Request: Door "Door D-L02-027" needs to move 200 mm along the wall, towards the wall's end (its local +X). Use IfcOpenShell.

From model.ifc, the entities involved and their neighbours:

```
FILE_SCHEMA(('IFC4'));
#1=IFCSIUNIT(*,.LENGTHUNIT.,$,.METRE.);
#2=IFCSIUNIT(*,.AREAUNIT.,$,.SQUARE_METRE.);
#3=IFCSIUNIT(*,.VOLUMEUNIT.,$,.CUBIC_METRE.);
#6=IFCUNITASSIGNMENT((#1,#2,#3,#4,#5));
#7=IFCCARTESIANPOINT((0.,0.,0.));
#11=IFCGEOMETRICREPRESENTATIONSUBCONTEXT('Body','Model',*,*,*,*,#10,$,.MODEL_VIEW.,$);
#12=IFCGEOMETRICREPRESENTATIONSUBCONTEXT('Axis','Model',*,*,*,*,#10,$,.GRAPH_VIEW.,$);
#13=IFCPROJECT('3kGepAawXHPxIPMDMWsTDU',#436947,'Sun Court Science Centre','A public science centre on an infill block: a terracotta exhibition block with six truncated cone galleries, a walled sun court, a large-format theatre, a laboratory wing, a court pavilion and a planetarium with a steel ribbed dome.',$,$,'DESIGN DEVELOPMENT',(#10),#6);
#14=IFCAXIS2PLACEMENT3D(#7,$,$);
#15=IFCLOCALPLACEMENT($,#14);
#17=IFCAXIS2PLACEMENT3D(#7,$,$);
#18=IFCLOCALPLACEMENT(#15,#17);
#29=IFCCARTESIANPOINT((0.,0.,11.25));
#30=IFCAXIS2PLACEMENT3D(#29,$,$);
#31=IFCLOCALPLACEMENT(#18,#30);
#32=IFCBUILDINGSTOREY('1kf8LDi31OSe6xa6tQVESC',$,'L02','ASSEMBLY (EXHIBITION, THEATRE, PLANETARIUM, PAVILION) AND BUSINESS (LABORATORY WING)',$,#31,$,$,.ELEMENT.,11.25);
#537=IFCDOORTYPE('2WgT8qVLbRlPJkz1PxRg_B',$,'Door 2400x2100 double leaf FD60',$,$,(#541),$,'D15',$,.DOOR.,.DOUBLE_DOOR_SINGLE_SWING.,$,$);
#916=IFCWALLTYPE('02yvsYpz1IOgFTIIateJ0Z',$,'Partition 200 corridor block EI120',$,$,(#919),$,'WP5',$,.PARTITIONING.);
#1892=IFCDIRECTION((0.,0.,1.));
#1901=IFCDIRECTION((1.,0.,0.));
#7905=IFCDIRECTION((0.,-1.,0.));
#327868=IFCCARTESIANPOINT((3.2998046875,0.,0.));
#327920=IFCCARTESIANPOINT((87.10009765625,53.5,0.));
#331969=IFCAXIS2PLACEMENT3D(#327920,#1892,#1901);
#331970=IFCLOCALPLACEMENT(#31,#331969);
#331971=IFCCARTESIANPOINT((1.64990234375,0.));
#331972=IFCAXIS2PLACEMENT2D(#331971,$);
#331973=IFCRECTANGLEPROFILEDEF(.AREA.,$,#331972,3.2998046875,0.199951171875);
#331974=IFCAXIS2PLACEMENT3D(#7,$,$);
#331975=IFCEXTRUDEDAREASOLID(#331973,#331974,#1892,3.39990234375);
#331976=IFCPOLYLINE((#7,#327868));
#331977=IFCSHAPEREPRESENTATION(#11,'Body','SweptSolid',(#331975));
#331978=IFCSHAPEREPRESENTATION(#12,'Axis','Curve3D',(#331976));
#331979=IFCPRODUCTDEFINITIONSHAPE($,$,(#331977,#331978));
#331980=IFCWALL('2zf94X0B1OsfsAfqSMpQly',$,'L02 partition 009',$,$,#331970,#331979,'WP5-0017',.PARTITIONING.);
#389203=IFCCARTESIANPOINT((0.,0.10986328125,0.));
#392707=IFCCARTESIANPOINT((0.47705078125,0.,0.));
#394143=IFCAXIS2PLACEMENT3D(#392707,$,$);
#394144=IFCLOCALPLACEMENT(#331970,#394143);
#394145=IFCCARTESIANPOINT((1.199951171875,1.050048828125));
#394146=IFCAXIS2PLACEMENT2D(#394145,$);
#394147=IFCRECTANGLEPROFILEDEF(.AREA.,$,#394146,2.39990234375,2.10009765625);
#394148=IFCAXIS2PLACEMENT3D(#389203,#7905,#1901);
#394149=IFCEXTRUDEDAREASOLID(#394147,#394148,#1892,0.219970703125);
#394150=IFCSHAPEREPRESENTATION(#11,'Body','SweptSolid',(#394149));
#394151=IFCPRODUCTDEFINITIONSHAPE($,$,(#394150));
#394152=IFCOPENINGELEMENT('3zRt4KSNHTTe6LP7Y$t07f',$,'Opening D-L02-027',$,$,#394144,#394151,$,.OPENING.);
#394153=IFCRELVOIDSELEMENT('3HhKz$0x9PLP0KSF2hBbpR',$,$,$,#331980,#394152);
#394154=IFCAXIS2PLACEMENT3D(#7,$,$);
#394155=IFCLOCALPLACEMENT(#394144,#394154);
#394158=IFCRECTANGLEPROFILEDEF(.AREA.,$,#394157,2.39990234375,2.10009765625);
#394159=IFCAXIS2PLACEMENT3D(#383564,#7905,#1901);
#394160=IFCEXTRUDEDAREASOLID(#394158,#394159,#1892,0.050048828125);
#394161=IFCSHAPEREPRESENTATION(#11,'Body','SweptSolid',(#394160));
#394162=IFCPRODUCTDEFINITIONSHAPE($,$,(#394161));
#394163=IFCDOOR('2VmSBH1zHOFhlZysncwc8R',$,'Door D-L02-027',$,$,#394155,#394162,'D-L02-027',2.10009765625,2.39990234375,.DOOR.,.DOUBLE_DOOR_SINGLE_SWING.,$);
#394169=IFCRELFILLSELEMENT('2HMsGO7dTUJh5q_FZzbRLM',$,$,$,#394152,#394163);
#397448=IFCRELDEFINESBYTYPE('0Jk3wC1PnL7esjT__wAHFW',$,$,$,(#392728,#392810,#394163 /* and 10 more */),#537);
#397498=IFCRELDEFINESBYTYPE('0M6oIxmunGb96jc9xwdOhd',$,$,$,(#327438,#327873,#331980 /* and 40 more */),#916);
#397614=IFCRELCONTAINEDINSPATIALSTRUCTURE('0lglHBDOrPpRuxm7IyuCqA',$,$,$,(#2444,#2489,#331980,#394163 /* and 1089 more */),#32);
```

```python
import ifcopenshell
import ifcopenshell.api.geometry
import ifcopenshell.util.placement

model = ifcopenshell.open("model.ifc")

door = model.by_guid("2VmSBH1zHOFhlZysncwc8R")
opening = door.FillsVoids[0].RelatingOpeningElement
wall = opening.VoidsElements[0].RelatingBuildingElement

wall_matrix = ifcopenshell.util.placement.get_local_placement(wall.ObjectPlacement)
shift = wall_matrix[:3, 0] * 0.2
before = ifcopenshell.util.placement.get_local_placement(door.ObjectPlacement)[:3, 3].copy()

# The door is placed relative to its opening, so it follows when the opening moves.
matrix = ifcopenshell.util.placement.get_local_placement(opening.ObjectPlacement)
matrix[:3, 3] += shift
ifcopenshell.api.geometry.edit_object_placement(
    model, product=opening, matrix=matrix, is_si=False, should_transform_children=True
)

after = ifcopenshell.util.placement.get_local_placement(door.ObjectPlacement)[:3, 3]
print("door moved by", (after - before).round(3) + 0.0)

model.write("model_v2.ifc")
```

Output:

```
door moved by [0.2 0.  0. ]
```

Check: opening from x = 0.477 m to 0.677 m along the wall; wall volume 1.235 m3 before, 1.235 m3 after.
